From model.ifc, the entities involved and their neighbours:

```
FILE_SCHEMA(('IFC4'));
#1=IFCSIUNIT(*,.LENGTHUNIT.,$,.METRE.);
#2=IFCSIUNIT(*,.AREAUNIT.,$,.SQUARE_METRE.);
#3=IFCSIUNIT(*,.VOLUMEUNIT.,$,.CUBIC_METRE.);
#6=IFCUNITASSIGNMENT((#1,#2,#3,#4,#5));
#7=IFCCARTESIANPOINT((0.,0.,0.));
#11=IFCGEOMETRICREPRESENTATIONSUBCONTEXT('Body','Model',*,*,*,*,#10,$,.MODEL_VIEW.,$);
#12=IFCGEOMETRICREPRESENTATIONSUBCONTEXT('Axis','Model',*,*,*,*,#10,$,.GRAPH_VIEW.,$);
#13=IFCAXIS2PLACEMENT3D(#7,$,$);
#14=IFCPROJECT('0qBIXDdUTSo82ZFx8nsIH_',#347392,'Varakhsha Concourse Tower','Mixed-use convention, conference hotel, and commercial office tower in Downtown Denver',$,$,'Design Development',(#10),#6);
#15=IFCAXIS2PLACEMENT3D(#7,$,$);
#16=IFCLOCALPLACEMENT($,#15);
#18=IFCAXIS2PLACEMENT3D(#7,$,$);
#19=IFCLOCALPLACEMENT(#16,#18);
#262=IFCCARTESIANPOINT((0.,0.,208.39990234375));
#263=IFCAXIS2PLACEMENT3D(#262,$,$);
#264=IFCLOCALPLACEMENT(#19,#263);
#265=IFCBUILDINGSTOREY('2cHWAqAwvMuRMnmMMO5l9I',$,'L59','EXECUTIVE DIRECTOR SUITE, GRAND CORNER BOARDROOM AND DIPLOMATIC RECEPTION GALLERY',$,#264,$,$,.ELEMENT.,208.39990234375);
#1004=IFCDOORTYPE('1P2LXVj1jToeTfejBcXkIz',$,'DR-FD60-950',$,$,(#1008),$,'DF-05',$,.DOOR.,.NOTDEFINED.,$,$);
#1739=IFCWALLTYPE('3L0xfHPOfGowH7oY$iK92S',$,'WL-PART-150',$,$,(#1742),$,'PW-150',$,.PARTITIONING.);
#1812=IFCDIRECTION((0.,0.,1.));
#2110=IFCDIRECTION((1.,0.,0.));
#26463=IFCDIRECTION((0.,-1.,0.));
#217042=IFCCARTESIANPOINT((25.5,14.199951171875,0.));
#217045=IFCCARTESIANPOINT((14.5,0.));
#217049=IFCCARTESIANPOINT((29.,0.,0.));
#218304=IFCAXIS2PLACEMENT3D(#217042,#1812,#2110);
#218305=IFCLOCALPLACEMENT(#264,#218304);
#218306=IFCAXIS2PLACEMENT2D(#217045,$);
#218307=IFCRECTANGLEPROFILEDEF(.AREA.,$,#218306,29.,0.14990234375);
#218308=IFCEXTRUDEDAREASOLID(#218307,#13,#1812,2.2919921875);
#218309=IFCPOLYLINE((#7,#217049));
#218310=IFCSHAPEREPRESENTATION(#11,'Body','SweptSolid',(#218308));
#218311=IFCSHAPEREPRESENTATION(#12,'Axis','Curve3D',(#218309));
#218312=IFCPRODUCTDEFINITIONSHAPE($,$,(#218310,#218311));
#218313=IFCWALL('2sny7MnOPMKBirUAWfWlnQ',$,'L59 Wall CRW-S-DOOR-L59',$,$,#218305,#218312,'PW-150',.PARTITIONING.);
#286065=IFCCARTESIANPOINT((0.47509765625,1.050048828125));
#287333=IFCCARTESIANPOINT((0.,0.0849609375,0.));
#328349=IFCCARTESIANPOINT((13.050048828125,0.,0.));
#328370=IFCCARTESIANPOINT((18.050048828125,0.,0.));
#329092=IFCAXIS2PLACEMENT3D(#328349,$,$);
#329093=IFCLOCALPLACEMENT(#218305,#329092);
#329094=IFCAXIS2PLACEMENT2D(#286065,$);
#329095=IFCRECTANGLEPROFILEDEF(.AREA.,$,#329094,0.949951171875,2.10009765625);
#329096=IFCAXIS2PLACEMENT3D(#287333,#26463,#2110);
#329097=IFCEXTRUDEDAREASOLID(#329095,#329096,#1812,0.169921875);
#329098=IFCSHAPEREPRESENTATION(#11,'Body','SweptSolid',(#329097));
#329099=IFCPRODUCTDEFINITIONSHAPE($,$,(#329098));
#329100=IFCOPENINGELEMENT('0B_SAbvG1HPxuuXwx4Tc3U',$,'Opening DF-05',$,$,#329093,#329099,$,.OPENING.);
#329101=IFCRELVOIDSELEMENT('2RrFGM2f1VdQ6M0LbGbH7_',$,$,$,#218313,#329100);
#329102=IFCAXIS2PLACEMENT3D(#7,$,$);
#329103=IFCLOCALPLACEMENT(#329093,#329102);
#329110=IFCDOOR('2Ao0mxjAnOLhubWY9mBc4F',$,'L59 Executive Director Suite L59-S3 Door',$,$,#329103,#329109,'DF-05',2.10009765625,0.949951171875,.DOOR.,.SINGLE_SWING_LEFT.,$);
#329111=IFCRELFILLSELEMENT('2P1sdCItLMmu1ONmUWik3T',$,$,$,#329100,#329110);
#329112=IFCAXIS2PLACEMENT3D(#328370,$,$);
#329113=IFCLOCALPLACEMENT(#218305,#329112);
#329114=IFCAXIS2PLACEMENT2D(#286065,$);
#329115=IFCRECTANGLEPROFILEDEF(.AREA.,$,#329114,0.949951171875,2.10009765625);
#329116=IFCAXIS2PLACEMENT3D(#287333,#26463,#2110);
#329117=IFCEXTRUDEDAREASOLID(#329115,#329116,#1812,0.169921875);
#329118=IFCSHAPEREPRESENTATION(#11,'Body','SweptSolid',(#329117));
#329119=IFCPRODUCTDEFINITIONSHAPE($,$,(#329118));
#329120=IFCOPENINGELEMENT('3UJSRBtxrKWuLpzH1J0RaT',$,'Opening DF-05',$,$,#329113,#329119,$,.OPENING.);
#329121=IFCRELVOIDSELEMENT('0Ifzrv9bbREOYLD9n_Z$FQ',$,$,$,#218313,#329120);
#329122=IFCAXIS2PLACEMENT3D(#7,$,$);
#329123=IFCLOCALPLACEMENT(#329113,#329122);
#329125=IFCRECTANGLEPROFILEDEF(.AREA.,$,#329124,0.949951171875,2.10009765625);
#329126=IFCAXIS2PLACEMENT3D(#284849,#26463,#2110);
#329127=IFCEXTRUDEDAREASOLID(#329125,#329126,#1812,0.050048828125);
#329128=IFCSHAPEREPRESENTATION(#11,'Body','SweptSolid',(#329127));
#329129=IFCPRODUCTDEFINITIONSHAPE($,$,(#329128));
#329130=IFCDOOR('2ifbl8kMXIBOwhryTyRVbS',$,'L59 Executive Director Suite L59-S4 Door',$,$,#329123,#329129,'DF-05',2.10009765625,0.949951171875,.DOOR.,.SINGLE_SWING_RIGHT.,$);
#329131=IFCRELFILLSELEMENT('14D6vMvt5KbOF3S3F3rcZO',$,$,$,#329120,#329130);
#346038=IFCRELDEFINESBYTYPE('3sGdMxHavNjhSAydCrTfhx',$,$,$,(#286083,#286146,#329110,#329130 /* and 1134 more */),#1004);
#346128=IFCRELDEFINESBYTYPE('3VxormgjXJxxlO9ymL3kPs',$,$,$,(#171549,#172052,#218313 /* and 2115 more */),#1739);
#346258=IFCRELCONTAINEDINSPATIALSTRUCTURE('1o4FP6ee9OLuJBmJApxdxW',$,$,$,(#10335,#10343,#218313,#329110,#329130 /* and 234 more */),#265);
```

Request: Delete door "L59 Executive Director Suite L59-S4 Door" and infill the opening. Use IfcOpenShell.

```python
import ifcopenshell
import ifcopenshell.api.feature
import ifcopenshell.api.root
import ifcopenshell.geom
import ifcopenshell.util.shape

model = ifcopenshell.open("model.ifc")
settings = ifcopenshell.geom.settings()


def volume(element):
    """Net volume in cubic metres, openings subtracted."""
    shape = ifcopenshell.geom.create_shape(settings, element)
    return ifcopenshell.util.shape.get_volume(shape.geometry)


door = model.by_guid("2ifbl8kMXIBOwhryTyRVbS")
opening = door.FillsVoids[0].RelatingOpeningElement
wall = opening.VoidsElements[0].RelatingBuildingElement
before = volume(wall)

ifcopenshell.api.root.remove_product(model, product=door)
ifcopenshell.api.feature.remove_feature(model, feature=opening)

after = volume(wall)

print(f"wall volume {before:.3f} -> {after:.3f} m3")

model.write("model_v2.ifc")
```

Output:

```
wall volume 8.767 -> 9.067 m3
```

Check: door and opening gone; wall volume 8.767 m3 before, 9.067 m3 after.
